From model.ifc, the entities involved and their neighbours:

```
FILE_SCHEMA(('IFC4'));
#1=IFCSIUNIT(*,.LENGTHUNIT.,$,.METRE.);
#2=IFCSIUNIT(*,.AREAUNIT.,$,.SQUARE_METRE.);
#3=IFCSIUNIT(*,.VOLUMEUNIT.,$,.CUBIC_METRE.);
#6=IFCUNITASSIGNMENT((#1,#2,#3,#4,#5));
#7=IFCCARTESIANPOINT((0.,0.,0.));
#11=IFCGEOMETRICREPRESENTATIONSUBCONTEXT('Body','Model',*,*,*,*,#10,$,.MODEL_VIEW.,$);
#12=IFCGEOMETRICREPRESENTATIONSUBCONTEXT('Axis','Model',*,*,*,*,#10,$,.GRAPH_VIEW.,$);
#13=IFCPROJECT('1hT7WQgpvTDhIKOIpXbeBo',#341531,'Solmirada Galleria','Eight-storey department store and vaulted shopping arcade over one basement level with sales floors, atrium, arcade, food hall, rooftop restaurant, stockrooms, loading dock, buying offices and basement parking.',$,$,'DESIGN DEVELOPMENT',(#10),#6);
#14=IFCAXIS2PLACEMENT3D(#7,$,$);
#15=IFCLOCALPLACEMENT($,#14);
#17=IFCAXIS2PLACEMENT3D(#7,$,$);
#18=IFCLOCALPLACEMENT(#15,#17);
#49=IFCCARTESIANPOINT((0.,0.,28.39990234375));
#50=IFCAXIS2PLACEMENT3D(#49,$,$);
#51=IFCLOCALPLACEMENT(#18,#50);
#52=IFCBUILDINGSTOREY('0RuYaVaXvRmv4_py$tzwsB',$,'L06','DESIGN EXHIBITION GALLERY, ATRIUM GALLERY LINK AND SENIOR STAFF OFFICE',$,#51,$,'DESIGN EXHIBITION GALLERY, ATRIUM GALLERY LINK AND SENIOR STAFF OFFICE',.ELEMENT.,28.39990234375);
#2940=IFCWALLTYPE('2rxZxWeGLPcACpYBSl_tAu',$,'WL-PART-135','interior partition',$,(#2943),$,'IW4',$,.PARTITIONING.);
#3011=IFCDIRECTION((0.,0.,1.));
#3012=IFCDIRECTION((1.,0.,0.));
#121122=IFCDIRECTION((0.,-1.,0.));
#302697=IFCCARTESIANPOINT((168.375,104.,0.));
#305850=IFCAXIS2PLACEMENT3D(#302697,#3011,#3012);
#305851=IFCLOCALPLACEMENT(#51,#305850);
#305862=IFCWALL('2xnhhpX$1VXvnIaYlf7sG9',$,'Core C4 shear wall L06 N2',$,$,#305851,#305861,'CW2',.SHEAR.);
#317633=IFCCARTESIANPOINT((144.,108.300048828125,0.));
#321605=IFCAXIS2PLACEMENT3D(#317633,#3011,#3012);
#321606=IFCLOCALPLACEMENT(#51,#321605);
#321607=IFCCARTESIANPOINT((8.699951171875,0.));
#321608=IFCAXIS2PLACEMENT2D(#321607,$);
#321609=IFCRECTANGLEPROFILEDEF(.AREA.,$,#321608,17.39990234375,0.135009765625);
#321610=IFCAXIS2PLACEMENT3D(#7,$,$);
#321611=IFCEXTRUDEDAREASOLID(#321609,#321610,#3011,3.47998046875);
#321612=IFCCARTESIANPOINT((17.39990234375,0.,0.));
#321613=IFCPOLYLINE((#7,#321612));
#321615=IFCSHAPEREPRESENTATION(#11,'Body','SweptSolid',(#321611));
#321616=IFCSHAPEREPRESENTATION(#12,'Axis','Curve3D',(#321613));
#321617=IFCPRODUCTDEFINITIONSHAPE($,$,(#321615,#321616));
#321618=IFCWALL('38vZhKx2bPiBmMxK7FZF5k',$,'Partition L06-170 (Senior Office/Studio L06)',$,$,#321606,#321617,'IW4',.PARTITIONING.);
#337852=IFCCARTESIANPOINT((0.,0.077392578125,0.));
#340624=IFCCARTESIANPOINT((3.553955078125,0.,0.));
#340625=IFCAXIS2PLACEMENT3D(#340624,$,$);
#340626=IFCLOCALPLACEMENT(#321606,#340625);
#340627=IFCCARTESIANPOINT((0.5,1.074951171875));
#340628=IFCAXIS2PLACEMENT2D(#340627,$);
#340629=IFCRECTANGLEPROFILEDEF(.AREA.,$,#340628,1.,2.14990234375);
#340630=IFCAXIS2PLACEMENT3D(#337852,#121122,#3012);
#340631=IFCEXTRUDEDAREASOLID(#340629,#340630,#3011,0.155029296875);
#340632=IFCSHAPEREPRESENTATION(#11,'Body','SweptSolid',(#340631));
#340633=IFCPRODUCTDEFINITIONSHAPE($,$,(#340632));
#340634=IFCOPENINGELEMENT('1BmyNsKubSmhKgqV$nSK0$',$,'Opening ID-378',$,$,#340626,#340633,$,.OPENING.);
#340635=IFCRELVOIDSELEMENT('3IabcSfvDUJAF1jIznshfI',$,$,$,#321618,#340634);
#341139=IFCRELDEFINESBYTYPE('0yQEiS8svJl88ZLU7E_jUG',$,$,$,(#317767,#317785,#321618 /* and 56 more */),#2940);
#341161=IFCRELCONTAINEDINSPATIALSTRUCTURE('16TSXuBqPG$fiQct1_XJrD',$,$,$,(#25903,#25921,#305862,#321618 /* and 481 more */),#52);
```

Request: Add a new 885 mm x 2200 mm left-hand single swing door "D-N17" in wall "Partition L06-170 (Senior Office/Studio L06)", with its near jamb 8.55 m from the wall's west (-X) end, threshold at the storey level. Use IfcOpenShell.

```python
import numpy as np
import ifcopenshell
import ifcopenshell.api.feature
import ifcopenshell.api.geometry
import ifcopenshell.api.root
import ifcopenshell.api.spatial
import ifcopenshell.geom
import ifcopenshell.util.element
import ifcopenshell.util.placement
import ifcopenshell.util.representation
import ifcopenshell.util.shape
import ifcopenshell.util.unit

model = ifcopenshell.open("model.ifc")
unit_scale = ifcopenshell.util.unit.calculate_unit_scale(model)
settings = ifcopenshell.geom.settings()


def volume(element):
    """Net volume in cubic metres, openings subtracted."""
    shape = ifcopenshell.geom.create_shape(settings, element)
    return ifcopenshell.util.shape.get_volume(shape.geometry)


wall = model.by_guid("38vZhKx2bPiBmMxK7FZF5k")
storey = ifcopenshell.util.element.get_container(wall, ifc_class="IfcBuildingStorey")
context = ifcopenshell.util.representation.get_context(model, "Model", "Body", "MODEL_VIEW")
before = volume(wall)

width, height, from_end, sill = 0.885, 2.2, 8.55, 0.0  # metres

# The wall runs along its own X axis, and the end named is its -X end.
wall_shape = ifcopenshell.geom.create_shape(settings, wall)
x, y, z = ifcopenshell.util.shape.get_vertices(wall_shape.geometry).T
start = x.min() + from_end
face, thickness = float(y.min()), float(y.max() - y.min())
wall_matrix = ifcopenshell.util.placement.get_local_placement(wall.ObjectPlacement)
level = ifcopenshell.util.placement.get_local_placement(storey.ObjectPlacement)[2, 3]


def in_wall(x, y):
    """Placement at x, y metres in the wall's axes, at sill height."""
    matrix = wall_matrix.copy()
    matrix[:, 3] = wall_matrix @ np.array([x / unit_scale, y / unit_scale, 0.0, 1.0])
    matrix[2, 3] = level + sill / unit_scale
    return matrix


# Opening: a box that overshoots both wall faces by 50 mm.
opening = ifcopenshell.api.root.create_entity(model, ifc_class="IfcOpeningElement", predefined_type="OPENING")
box = ifcopenshell.api.geometry.add_wall_representation(
    model, context=context, length=width, height=height, thickness=thickness + 0.1
)
ifcopenshell.api.geometry.assign_representation(model, product=opening, representation=box)
ifcopenshell.api.geometry.edit_object_placement(model, product=opening, matrix=in_wall(start, face - 0.05), is_si=False)
ifcopenshell.api.feature.add_feature(model, feature=opening, element=wall)

door = ifcopenshell.api.root.create_entity(model, ifc_class="IfcDoor", name="D-N17", predefined_type="DOOR")
door.OverallWidth, door.OverallHeight = width / unit_scale, height / unit_scale
door.OperationType = "SINGLE_SWING_LEFT"
body = ifcopenshell.api.geometry.add_door_representation(
    model,
    context=context,
    overall_width=door.OverallWidth,
    overall_height=door.OverallHeight,
    operation_type="SINGLE_SWING_LEFT",
    lining_properties={"LiningDepth": thickness / unit_scale, "ThresholdDepth": thickness / unit_scale},
)
ifcopenshell.api.geometry.assign_representation(model, product=door, representation=body)
ifcopenshell.api.spatial.assign_container(model, products=[door], relating_structure=storey)
ifcopenshell.api.feature.add_filling(model, opening=opening, element=door)

# The lining spans the wall, so the door starts at the wall face.
ifcopenshell.api.geometry.edit_object_placement(model, product=door, matrix=in_wall(start, face), is_si=False)

after = volume(wall)

print(f"wall volume {before:.3f} -> {after:.3f} m3")

model.write("model-out.ifc")
```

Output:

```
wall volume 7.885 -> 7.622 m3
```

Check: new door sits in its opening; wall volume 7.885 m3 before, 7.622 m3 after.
